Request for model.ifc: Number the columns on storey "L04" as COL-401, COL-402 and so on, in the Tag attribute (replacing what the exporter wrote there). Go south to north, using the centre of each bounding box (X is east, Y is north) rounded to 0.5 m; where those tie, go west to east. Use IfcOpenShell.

First a look at what the model holds.

```python
import ifcopenshell
import ifcopenshell.util.element
import ifcopenshell.util.placement

model = ifcopenshell.open("model.ifc")
print(model.schema)
storey = next(s for s in model.by_type("IfcBuildingStorey") if s.Name == "L04")
columns = [e for e in ifcopenshell.util.element.get_decomposition(storey) if e.is_a("IfcColumn")]
for e in sorted(columns, key=lambda e: e.id()):
    origin = ifcopenshell.util.placement.get_local_placement(e.ObjectPlacement)[:3, 3]
    print(e.id(), e.Tag, e.Name, origin.round(2) + 0.0, sep=" | ")
```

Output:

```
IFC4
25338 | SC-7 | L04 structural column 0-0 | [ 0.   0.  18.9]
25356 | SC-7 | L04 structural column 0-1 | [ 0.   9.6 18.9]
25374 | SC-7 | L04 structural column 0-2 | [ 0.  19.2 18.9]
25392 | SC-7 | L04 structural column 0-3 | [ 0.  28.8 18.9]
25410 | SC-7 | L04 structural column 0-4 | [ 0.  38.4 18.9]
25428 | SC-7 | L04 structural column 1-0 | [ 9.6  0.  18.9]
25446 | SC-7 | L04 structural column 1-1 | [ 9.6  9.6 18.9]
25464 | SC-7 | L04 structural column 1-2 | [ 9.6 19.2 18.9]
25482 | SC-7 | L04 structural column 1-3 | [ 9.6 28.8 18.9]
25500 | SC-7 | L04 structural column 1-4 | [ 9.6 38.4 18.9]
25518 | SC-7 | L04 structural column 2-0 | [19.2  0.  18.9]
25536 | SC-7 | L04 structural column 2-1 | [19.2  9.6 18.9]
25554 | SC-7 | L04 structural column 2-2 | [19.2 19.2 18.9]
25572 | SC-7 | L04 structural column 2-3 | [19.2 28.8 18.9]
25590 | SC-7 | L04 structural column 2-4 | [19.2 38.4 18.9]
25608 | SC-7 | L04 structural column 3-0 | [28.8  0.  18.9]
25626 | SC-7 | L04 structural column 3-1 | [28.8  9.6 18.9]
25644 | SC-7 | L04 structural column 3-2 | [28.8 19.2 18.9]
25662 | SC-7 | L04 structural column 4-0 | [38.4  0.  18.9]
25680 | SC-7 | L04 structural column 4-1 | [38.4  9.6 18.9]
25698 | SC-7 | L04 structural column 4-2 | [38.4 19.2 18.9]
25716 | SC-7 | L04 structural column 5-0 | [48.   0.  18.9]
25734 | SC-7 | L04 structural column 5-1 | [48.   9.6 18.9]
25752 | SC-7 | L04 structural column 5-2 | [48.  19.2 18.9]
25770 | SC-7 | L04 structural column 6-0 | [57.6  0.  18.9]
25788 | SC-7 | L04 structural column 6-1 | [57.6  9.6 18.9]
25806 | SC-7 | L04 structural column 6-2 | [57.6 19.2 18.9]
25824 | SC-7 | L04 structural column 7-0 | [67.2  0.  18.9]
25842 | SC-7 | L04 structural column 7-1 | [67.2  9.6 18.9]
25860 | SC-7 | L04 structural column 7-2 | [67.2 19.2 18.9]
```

```python
import ifcopenshell
import ifcopenshell.geom
import ifcopenshell.util.element
import ifcopenshell.util.shape

model = ifcopenshell.open("model.ifc")
settings = ifcopenshell.geom.settings()
settings.set("use-world-coords", True)


def centre(element):
    shape = ifcopenshell.geom.create_shape(settings, element)
    return ifcopenshell.util.shape.get_bbox_centroid(shape.geometry)


storey = next(s for s in model.by_type("IfcBuildingStorey") if s.Name == "L04")
columns = [e for e in ifcopenshell.util.element.get_decomposition(storey) if e.is_a("IfcColumn")]

# Insertion points can sit at a corner or the storey origin, so sort by the geometry (in metres).
centres = {e: centre(e) for e in columns}
columns.sort(key=lambda e: (round(centres[e][1] / 0.5), centres[e][0]))

for i, e in enumerate(columns, start=1):
    number = f"COL-4{i:02d}"
    e.Tag = number
    print(e.id(), number)

model.write("model-out.ifc")
```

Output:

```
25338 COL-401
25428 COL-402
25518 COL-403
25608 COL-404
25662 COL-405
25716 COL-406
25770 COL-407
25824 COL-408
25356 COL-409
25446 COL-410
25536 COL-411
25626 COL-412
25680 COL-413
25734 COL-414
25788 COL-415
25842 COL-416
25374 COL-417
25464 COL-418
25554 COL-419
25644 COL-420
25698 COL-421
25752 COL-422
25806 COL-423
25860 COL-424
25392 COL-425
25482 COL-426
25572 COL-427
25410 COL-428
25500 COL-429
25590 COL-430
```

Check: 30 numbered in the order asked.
